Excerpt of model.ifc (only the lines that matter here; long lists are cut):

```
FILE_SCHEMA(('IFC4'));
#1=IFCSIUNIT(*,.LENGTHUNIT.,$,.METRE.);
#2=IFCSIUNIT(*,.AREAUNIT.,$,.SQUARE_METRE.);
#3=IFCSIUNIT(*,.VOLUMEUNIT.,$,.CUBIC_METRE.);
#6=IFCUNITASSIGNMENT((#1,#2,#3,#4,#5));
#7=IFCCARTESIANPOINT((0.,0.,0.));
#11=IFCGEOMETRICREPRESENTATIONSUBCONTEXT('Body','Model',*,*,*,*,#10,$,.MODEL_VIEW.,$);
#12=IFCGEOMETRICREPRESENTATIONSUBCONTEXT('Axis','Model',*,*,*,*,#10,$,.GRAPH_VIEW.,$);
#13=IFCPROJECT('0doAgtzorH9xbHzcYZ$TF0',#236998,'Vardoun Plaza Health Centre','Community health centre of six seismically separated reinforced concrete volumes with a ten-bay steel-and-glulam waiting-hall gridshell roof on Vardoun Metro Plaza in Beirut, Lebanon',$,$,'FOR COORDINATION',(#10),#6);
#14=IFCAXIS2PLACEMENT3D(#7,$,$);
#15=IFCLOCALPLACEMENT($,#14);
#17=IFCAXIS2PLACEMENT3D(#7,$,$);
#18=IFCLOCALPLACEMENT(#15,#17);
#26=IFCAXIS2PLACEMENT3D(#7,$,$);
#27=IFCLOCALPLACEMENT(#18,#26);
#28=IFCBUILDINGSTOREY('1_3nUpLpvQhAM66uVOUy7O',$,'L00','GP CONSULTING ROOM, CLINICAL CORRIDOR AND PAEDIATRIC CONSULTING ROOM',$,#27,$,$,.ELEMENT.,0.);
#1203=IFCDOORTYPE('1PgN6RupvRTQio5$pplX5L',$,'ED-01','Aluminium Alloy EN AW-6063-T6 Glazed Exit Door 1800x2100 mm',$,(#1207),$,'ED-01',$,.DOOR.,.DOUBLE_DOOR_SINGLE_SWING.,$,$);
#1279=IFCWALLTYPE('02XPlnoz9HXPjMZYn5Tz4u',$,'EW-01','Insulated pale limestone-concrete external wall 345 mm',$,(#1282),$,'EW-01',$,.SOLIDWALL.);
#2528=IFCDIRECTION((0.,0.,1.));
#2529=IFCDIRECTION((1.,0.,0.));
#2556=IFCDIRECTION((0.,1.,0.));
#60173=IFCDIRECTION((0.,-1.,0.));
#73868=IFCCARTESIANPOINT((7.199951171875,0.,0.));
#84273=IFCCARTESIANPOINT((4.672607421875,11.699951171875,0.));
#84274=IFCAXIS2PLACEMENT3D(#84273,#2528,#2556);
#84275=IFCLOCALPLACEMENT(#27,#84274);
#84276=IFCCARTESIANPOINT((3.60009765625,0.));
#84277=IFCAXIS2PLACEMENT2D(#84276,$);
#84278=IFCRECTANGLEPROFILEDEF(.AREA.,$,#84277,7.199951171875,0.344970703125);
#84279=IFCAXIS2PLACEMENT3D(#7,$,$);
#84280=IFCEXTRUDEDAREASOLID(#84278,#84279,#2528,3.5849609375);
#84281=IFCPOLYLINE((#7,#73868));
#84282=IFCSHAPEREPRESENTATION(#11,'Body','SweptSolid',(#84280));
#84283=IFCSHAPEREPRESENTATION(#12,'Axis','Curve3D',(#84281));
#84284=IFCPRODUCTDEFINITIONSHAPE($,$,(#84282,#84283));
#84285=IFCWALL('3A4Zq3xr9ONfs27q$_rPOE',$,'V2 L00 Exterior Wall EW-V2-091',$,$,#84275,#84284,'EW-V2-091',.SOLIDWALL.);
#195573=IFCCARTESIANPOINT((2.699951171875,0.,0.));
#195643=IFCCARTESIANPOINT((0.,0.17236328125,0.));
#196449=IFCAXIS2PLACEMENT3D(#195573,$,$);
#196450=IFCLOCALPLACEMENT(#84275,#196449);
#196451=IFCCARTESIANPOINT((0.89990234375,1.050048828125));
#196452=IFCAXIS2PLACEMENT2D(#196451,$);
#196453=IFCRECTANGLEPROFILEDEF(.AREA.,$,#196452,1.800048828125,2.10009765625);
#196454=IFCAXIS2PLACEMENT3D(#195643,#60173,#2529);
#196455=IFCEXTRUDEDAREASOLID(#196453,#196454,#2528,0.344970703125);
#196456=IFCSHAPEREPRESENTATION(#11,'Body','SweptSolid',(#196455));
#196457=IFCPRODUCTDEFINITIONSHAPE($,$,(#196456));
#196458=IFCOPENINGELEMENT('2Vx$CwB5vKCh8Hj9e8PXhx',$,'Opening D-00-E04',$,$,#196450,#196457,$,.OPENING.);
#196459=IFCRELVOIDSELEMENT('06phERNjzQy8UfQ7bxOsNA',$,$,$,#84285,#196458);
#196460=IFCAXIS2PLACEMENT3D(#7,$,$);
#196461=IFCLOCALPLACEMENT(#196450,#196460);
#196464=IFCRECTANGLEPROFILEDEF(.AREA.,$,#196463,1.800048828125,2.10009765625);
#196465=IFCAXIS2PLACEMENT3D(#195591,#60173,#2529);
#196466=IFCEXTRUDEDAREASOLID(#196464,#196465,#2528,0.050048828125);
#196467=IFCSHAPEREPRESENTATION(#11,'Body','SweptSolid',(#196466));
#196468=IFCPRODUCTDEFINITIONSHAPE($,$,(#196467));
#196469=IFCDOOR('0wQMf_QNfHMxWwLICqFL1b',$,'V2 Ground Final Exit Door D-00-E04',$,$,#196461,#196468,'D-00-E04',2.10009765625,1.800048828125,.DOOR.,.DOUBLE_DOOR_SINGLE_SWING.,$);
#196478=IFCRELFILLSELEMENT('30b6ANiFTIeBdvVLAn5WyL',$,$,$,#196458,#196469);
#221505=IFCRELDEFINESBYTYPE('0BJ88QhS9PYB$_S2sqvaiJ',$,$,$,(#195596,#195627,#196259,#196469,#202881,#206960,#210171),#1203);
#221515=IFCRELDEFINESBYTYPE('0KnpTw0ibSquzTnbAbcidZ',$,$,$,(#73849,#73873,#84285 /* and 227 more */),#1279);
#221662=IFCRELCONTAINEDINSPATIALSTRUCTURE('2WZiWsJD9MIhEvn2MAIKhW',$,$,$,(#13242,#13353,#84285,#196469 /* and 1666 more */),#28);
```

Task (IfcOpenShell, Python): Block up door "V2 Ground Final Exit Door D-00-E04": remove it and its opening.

```python
import ifcopenshell
import ifcopenshell.api.feature
import ifcopenshell.api.root
import ifcopenshell.geom
import ifcopenshell.util.shape

model = ifcopenshell.open("model.ifc")
settings = ifcopenshell.geom.settings()


def volume(element):
    """Net volume in cubic metres, openings subtracted."""
    shape = ifcopenshell.geom.create_shape(settings, element)
    return ifcopenshell.util.shape.get_volume(shape.geometry)


door = model.by_guid("0wQMf_QNfHMxWwLICqFL1b")
opening = door.FillsVoids[0].RelatingOpeningElement
wall = opening.VoidsElements[0].RelatingBuildingElement
before = volume(wall)

ifcopenshell.api.root.remove_product(model, product=door)
ifcopenshell.api.feature.remove_feature(model, feature=opening)

after = volume(wall)

print(f"wall volume {before:.3f} -> {after:.3f} m3")

model.write("model_v2.ifc")
```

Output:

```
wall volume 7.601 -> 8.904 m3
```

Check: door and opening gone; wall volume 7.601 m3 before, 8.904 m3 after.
